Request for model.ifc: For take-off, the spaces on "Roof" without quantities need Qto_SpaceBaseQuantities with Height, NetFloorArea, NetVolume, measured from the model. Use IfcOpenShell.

First a look at what the model holds.

```python
import ifcopenshell
import ifcopenshell.util.element
import ifcopenshell.util.unit

model = ifcopenshell.open("model.ifc")
print(model.schema)
for unit_type in ("LENGTHUNIT", "AREAUNIT", "VOLUMEUNIT"):
    print(unit_type, ifcopenshell.util.unit.calculate_unit_scale(model, unit_type))
storey = next(s for s in model.by_type("IfcBuildingStorey") if s.Name == "Roof")
spaces = [e for e in ifcopenshell.util.element.get_decomposition(storey) if e.is_a("IfcSpace")]
for e in sorted(spaces, key=lambda e: e.id()):
    print(e.id(), e.is_a(), e.Name, list(ifcopenshell.util.element.get_psets(e, qtos_only=True)), sep=" | ")
```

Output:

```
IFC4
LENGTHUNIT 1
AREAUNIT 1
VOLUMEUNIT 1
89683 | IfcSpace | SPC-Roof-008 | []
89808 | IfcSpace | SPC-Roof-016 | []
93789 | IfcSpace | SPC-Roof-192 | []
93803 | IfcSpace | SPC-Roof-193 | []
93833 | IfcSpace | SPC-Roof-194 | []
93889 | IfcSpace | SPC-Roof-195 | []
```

```python
import ifcopenshell
import ifcopenshell.api.pset
import ifcopenshell.geom
import ifcopenshell.util.element
import ifcopenshell.util.shape
import ifcopenshell.util.unit

model = ifcopenshell.open("model.ifc")
unit_scale = ifcopenshell.util.unit.calculate_unit_scale(model)
area_scale = ifcopenshell.util.unit.calculate_unit_scale(model, "AREAUNIT")
volume_scale = ifcopenshell.util.unit.calculate_unit_scale(model, "VOLUMEUNIT")
settings = ifcopenshell.geom.settings()

storey = next(s for s in model.by_type("IfcBuildingStorey") if s.Name == "Roof")
spaces = [e for e in ifcopenshell.util.element.get_decomposition(storey) if e.is_a("IfcSpace")]

for e in sorted(spaces, key=lambda e: e.id()):
    if ifcopenshell.util.element.get_psets(e, qtos_only=True, should_inherit=False):
        continue
    # Geometry comes back in metres, in the element's own axes.
    shape = ifcopenshell.geom.create_shape(settings, e)
    values = {
        "Height": ifcopenshell.util.shape.get_z(shape.geometry) / unit_scale,
        "NetFloorArea": ifcopenshell.util.shape.get_footprint_area(shape.geometry) / area_scale,
        "NetVolume": ifcopenshell.util.shape.get_volume(shape.geometry) / volume_scale,
    }
    qto = ifcopenshell.api.pset.add_qto(model, product=e, name="Qto_SpaceBaseQuantities")
    ifcopenshell.api.pset.edit_qto(model, qto=qto, properties=values)
    print(e.id(), {k: round(v, 3) for k, v in values.items()})

model.write("model_updated.ifc")
```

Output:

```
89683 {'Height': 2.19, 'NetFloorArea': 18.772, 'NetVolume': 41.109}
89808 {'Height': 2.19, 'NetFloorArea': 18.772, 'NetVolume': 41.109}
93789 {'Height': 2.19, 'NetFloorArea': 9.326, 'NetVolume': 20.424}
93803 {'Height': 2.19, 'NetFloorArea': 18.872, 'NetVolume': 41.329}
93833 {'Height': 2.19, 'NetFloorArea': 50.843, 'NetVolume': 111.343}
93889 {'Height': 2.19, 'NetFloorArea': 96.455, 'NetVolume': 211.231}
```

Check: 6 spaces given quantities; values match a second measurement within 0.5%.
